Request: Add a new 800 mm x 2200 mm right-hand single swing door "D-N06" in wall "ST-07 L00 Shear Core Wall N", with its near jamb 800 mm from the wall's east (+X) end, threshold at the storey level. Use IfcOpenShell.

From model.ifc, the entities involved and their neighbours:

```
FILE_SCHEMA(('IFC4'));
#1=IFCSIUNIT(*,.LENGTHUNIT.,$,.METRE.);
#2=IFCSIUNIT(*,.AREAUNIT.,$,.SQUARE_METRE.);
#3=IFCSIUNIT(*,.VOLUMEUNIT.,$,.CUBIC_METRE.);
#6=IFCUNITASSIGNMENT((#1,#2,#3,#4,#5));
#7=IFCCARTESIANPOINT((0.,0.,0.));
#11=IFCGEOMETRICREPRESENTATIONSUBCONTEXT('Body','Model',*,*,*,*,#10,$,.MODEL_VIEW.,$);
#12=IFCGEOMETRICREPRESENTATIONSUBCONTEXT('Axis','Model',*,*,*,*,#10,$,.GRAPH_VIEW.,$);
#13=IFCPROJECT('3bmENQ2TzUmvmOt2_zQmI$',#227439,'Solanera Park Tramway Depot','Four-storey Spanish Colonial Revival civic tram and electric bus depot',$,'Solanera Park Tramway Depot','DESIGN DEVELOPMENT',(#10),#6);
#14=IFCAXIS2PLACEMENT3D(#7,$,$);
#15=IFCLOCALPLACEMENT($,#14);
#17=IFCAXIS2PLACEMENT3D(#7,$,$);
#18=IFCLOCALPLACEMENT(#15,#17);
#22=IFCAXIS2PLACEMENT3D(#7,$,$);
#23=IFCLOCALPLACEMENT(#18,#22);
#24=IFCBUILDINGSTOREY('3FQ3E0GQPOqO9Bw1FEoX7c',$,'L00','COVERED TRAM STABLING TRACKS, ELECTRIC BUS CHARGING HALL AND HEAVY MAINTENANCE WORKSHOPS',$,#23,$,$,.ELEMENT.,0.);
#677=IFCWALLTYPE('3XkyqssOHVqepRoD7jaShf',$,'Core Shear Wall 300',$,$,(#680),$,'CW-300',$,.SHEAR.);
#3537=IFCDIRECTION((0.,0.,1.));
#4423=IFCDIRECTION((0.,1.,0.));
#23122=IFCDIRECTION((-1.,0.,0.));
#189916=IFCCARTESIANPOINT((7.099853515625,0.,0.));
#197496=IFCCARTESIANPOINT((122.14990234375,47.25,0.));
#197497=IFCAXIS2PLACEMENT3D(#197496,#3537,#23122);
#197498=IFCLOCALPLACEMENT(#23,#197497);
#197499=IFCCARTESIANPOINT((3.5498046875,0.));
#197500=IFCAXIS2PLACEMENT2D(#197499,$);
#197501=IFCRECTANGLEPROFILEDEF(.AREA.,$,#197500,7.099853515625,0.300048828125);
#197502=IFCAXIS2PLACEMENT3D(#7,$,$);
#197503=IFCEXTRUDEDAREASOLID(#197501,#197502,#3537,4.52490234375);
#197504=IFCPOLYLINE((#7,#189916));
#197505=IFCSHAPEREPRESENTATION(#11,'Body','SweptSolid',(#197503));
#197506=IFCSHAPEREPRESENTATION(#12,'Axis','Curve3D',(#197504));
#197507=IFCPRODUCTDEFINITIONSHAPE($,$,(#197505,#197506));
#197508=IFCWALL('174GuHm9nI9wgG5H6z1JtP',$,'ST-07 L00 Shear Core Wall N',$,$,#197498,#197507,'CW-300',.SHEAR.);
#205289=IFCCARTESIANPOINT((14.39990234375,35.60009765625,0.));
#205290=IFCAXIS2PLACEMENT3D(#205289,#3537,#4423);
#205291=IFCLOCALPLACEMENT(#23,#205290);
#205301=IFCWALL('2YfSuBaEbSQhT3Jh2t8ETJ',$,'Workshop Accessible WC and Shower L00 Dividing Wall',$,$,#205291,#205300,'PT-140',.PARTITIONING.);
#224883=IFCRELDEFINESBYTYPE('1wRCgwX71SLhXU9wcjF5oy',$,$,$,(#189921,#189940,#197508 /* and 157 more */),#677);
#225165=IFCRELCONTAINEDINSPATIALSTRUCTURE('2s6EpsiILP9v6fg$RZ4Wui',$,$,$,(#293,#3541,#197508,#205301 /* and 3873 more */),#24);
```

```python
import numpy as np
import ifcopenshell
import ifcopenshell.api.feature
import ifcopenshell.api.geometry
import ifcopenshell.api.root
import ifcopenshell.api.spatial
import ifcopenshell.geom
import ifcopenshell.util.element
import ifcopenshell.util.placement
import ifcopenshell.util.representation
import ifcopenshell.util.shape
import ifcopenshell.util.unit

model = ifcopenshell.open("model.ifc")
unit_scale = ifcopenshell.util.unit.calculate_unit_scale(model)
settings = ifcopenshell.geom.settings()


def volume(element):
    """Net volume in cubic metres, openings subtracted."""
    shape = ifcopenshell.geom.create_shape(settings, element)
    return ifcopenshell.util.shape.get_volume(shape.geometry)


wall = model.by_guid("174GuHm9nI9wgG5H6z1JtP")
storey = ifcopenshell.util.element.get_container(wall, ifc_class="IfcBuildingStorey")
context = ifcopenshell.util.representation.get_context(model, "Model", "Body", "MODEL_VIEW")
before = volume(wall)

width, height, from_end, sill = 0.8, 2.2, 0.8, 0.0  # metres

# The wall runs along its own X axis, and the end named is its -X end.
wall_shape = ifcopenshell.geom.create_shape(settings, wall)
x, y, z = ifcopenshell.util.shape.get_vertices(wall_shape.geometry).T
start = x.min() + from_end
face, thickness = float(y.min()), float(y.max() - y.min())
wall_matrix = ifcopenshell.util.placement.get_local_placement(wall.ObjectPlacement)
level = ifcopenshell.util.placement.get_local_placement(storey.ObjectPlacement)[2, 3]


def in_wall(x, y):
    """Placement at x, y metres in the wall's axes, at sill height."""
    matrix = wall_matrix.copy()
    matrix[:, 3] = wall_matrix @ np.array([x / unit_scale, y / unit_scale, 0.0, 1.0])
    matrix[2, 3] = level + sill / unit_scale
    return matrix


# Opening: a box that overshoots both wall faces by 50 mm.
opening = ifcopenshell.api.root.create_entity(model, ifc_class="IfcOpeningElement", predefined_type="OPENING")
box = ifcopenshell.api.geometry.add_wall_representation(
    model, context=context, length=width, height=height, thickness=thickness + 0.1
)
ifcopenshell.api.geometry.assign_representation(model, product=opening, representation=box)
ifcopenshell.api.geometry.edit_object_placement(model, product=opening, matrix=in_wall(start, face - 0.05), is_si=False)
ifcopenshell.api.feature.add_feature(model, feature=opening, element=wall)

door = ifcopenshell.api.root.create_entity(model, ifc_class="IfcDoor", name="D-N06", predefined_type="DOOR")
door.OverallWidth, door.OverallHeight = width / unit_scale, height / unit_scale
door.OperationType = "SINGLE_SWING_RIGHT"
body = ifcopenshell.api.geometry.add_door_representation(
    model,
    context=context,
    overall_width=door.OverallWidth,
    overall_height=door.OverallHeight,
    operation_type="SINGLE_SWING_RIGHT",
    lining_properties={"LiningDepth": thickness / unit_scale, "ThresholdDepth": thickness / unit_scale},
)
ifcopenshell.api.geometry.assign_representation(model, product=door, representation=body)
ifcopenshell.api.spatial.assign_container(model, products=[door], relating_structure=storey)
ifcopenshell.api.feature.add_filling(model, opening=opening, element=door)

# The lining spans the wall, so the door starts at the wall face.
ifcopenshell.api.geometry.edit_object_placement(model, product=door, matrix=in_wall(start, face), is_si=False)

after = volume(wall)

print(f"wall volume {before:.3f} -> {after:.3f} m3")

model.write("model-out.ifc")
```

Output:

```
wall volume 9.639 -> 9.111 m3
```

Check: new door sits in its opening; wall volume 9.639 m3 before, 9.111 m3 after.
